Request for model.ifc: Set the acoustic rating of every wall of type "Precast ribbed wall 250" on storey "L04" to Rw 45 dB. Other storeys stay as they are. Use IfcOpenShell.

First a look at what the model holds.

```python
import ifcopenshell
import ifcopenshell.util.element

model = ifcopenshell.open("model.ifc")
print(model.schema)
storey = next(s for s in model.by_type("IfcBuildingStorey") if s.Name == "L04")
walls = [e for e in ifcopenshell.util.element.get_decomposition(storey) if e.is_a("IfcWall")]
seen = {}
for e in walls:
    element_type = ifcopenshell.util.element.get_type(e)
    key = (element_type.Name if element_type != e and element_type else None, ifcopenshell.util.element.get_pset(e, "Pset_WallCommon", "AcousticRating"))
    seen[key] = seen.get(key, 0) + 1
for (name, value), count in sorted(seen.items(), key=str):
    print(count, "x", name, "|", value)
```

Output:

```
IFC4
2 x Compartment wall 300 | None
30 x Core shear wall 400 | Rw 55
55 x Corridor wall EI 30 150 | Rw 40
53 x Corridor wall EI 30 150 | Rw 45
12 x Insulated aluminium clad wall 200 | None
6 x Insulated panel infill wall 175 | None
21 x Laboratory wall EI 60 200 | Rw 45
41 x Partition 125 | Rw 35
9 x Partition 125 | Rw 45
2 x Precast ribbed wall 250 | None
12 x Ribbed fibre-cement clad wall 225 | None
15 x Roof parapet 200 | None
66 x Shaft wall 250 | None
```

```python
import ifcopenshell
import ifcopenshell.api.pset
import ifcopenshell.util.element

model = ifcopenshell.open("model.ifc")

storey = next(s for s in model.by_type("IfcBuildingStorey") if s.Name == "L04")
walls = [e for e in ifcopenshell.util.element.get_decomposition(storey) if e.is_a("IfcWall")]

count = 0
for e in walls:
    element_type = ifcopenshell.util.element.get_type(e)
    if element_type in (None, e) or element_type.Name != "Precast ribbed wall 250":
        continue
    found = ifcopenshell.util.element.get_pset(e, "Pset_WallCommon", should_inherit=False)
    if found:
        pset = model.by_id(found["id"])
        if len(ifcopenshell.util.element.get_elements_by_pset(pset)) > 1:
            pset = ifcopenshell.api.pset.unshare_pset(model, products=[e], pset=pset)[0]
    else:
        pset = ifcopenshell.api.pset.add_pset(model, product=e, name="Pset_WallCommon")
    ifcopenshell.api.pset.edit_pset(model, pset=pset, properties={"AcousticRating": "Rw 45 dB"})
    count += 1

print(count, "walls updated")

model.write("model_edited.ifc")
```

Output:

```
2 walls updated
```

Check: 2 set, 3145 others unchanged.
